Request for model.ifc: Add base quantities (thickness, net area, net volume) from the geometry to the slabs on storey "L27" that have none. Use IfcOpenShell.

First a look at what the model holds.

```python
import ifcopenshell
import ifcopenshell.util.element
import ifcopenshell.util.unit

model = ifcopenshell.open("model.ifc")
print(model.schema)
for unit_type in ("LENGTHUNIT", "AREAUNIT", "VOLUMEUNIT"):
    print(unit_type, ifcopenshell.util.unit.calculate_unit_scale(model, unit_type))
storey = next(s for s in model.by_type("IfcBuildingStorey") if s.Name == "L27")
slabs = [e for e in ifcopenshell.util.element.get_decomposition(storey) if e.is_a("IfcSlab")]
for e in sorted(slabs, key=lambda e: e.id()):
    print(e.id(), e.is_a(), e.Name, list(ifcopenshell.util.element.get_psets(e, qtos_only=True)), sep=" | ")
```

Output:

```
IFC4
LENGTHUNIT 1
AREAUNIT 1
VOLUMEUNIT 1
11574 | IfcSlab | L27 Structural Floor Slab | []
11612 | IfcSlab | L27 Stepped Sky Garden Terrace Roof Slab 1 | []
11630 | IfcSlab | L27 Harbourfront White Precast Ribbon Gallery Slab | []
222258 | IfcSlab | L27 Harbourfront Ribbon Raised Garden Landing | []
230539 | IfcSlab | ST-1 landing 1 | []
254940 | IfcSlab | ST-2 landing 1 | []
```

```python
import ifcopenshell
import ifcopenshell.api.pset
import ifcopenshell.geom
import ifcopenshell.util.element
import ifcopenshell.util.shape
import ifcopenshell.util.unit

model = ifcopenshell.open("model.ifc")
unit_scale = ifcopenshell.util.unit.calculate_unit_scale(model)
area_scale = ifcopenshell.util.unit.calculate_unit_scale(model, "AREAUNIT")
volume_scale = ifcopenshell.util.unit.calculate_unit_scale(model, "VOLUMEUNIT")
settings = ifcopenshell.geom.settings()

storey = next(s for s in model.by_type("IfcBuildingStorey") if s.Name == "L27")
slabs = [e for e in ifcopenshell.util.element.get_decomposition(storey) if e.is_a("IfcSlab")]

for e in sorted(slabs, key=lambda e: e.id()):
    if ifcopenshell.util.element.get_psets(e, qtos_only=True, should_inherit=False):
        continue
    # Geometry comes back in metres, in the element's own axes.
    shape = ifcopenshell.geom.create_shape(settings, e)
    values = {
        "Width": ifcopenshell.util.shape.get_z(shape.geometry) / unit_scale,
        "NetArea": ifcopenshell.util.shape.get_footprint_area(shape.geometry) / area_scale,
        "NetVolume": ifcopenshell.util.shape.get_volume(shape.geometry) / volume_scale,
    }
    qto = ifcopenshell.api.pset.add_qto(model, product=e, name="Qto_SlabBaseQuantities")
    ifcopenshell.api.pset.edit_qto(model, qto=qto, properties=values)
    print(e.id(), {k: round(v, 3) for k, v in values.items()})

model.write("model-out.ifc")
```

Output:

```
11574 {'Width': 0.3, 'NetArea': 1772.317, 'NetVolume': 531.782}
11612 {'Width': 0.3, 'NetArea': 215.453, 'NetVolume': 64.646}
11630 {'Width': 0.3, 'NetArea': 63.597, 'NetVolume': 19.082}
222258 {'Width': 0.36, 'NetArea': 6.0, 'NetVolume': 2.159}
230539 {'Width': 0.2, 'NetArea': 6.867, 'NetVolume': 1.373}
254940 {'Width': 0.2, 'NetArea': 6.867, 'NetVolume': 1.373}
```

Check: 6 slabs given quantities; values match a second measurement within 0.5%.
